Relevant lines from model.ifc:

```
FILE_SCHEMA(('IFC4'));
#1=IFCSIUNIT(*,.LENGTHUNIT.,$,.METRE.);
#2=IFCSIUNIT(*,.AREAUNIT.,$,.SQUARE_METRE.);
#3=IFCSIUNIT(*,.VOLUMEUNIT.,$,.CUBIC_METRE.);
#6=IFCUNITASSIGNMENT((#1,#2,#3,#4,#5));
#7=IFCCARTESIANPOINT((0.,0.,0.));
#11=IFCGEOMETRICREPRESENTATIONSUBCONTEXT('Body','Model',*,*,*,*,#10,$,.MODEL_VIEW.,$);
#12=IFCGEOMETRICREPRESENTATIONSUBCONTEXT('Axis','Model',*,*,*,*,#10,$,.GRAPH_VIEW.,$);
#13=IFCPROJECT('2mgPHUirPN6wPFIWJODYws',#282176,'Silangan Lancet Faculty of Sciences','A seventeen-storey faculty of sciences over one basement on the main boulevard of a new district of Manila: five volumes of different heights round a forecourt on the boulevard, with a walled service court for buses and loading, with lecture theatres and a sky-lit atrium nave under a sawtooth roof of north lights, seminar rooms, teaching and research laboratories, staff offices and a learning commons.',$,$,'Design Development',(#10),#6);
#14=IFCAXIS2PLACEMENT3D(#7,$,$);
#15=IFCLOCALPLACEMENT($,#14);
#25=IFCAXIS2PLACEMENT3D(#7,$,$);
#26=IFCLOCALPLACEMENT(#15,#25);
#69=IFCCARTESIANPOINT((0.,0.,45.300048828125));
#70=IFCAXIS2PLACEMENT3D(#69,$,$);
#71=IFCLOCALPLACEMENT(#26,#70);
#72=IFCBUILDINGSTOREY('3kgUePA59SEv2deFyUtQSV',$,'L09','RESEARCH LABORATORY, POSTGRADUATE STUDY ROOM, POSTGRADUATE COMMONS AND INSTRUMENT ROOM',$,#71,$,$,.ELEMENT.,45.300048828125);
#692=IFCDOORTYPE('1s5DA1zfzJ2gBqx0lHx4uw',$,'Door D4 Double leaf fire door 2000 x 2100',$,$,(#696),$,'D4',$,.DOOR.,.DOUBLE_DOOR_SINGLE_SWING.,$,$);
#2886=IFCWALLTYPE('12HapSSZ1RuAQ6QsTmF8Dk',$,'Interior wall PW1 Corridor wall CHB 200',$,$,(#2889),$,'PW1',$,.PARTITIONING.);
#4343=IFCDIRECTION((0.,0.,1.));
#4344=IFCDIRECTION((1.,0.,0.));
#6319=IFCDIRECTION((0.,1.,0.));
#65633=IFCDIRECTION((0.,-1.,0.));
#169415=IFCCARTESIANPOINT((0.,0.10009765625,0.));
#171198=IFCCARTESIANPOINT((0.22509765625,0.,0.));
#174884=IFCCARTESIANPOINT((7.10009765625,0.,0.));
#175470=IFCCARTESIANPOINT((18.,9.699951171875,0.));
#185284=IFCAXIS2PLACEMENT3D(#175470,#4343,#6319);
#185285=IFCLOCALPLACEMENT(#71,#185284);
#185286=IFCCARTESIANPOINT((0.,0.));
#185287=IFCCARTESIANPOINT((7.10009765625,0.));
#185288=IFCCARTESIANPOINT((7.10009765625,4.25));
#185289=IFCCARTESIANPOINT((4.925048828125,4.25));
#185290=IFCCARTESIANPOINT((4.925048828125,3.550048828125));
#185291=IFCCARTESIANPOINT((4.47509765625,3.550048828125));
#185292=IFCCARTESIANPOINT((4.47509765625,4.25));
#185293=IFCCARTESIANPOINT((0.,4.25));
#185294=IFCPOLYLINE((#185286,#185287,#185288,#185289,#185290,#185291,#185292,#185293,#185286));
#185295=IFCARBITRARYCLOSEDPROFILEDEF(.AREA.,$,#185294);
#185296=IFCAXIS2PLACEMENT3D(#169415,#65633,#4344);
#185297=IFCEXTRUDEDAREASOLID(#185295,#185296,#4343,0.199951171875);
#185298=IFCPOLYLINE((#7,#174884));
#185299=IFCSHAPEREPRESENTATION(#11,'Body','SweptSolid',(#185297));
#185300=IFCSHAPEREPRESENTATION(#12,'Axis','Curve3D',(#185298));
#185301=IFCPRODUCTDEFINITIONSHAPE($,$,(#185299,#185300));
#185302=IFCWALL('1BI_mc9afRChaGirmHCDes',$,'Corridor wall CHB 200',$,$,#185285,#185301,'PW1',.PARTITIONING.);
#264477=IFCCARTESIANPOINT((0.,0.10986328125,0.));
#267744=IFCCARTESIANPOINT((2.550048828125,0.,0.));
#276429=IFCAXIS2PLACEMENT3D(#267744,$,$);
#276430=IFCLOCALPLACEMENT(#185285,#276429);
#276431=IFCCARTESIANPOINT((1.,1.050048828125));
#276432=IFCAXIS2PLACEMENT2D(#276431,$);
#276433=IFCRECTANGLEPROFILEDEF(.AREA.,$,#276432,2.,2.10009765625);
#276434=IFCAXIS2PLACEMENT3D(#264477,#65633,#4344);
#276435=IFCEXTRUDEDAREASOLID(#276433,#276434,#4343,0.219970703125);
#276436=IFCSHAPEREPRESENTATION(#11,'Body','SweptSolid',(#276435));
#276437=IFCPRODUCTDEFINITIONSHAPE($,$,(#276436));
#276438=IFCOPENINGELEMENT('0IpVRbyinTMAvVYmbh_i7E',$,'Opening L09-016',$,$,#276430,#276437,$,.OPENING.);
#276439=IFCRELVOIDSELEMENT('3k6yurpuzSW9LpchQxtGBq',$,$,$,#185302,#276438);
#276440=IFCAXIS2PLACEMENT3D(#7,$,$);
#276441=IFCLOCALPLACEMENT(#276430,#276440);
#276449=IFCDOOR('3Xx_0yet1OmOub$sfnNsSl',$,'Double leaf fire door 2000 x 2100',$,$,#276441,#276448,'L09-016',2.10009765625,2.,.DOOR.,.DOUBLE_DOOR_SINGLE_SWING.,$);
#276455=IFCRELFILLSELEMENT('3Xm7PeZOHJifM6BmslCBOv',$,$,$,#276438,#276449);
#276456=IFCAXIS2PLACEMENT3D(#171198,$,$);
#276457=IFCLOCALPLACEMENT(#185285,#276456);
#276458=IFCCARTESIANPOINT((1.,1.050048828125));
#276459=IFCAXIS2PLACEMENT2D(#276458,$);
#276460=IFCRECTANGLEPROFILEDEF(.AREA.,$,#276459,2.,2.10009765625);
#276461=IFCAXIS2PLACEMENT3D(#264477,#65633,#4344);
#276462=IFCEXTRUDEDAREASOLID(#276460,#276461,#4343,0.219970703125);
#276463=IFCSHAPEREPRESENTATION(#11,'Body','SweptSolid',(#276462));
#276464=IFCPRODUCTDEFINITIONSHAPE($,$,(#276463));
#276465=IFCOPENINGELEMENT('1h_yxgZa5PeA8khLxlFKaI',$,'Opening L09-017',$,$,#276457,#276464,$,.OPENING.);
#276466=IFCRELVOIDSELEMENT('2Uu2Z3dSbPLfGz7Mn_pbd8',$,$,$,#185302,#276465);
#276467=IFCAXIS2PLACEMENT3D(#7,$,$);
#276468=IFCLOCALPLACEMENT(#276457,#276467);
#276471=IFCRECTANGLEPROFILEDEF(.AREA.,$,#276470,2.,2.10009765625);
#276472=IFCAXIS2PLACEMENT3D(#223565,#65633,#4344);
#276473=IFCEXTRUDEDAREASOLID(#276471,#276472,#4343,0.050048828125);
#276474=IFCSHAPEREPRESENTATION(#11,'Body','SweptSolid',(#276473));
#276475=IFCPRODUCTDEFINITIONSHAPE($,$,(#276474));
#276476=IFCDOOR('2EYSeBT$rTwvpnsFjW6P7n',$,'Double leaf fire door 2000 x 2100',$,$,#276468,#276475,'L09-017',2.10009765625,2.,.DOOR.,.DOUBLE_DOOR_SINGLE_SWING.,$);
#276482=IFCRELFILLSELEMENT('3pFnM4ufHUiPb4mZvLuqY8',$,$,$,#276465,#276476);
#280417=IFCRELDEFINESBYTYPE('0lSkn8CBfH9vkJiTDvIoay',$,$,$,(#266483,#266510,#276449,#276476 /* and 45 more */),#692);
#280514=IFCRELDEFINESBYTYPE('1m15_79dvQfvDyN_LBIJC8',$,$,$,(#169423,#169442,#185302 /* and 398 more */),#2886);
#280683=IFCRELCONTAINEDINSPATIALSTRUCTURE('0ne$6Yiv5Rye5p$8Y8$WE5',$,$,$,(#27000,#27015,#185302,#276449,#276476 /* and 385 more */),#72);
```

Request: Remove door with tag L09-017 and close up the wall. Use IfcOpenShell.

```python
import ifcopenshell
import ifcopenshell.api.feature
import ifcopenshell.api.root
import ifcopenshell.geom
import ifcopenshell.util.shape

model = ifcopenshell.open("model.ifc")
settings = ifcopenshell.geom.settings()


def volume(element):
    """Net volume in cubic metres, openings subtracted."""
    shape = ifcopenshell.geom.create_shape(settings, element)
    return ifcopenshell.util.shape.get_volume(shape.geometry)


door = model.by_id(276476)
opening = door.FillsVoids[0].RelatingOpeningElement
wall = opening.VoidsElements[0].RelatingBuildingElement
before = volume(wall)

ifcopenshell.api.root.remove_product(model, product=door)
ifcopenshell.api.feature.remove_feature(model, feature=opening)

after = volume(wall)

print(f"wall volume {before:.3f} -> {after:.3f} m3")

model.write("model_rev.ifc")
```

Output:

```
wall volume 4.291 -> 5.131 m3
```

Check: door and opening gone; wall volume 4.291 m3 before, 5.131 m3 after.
